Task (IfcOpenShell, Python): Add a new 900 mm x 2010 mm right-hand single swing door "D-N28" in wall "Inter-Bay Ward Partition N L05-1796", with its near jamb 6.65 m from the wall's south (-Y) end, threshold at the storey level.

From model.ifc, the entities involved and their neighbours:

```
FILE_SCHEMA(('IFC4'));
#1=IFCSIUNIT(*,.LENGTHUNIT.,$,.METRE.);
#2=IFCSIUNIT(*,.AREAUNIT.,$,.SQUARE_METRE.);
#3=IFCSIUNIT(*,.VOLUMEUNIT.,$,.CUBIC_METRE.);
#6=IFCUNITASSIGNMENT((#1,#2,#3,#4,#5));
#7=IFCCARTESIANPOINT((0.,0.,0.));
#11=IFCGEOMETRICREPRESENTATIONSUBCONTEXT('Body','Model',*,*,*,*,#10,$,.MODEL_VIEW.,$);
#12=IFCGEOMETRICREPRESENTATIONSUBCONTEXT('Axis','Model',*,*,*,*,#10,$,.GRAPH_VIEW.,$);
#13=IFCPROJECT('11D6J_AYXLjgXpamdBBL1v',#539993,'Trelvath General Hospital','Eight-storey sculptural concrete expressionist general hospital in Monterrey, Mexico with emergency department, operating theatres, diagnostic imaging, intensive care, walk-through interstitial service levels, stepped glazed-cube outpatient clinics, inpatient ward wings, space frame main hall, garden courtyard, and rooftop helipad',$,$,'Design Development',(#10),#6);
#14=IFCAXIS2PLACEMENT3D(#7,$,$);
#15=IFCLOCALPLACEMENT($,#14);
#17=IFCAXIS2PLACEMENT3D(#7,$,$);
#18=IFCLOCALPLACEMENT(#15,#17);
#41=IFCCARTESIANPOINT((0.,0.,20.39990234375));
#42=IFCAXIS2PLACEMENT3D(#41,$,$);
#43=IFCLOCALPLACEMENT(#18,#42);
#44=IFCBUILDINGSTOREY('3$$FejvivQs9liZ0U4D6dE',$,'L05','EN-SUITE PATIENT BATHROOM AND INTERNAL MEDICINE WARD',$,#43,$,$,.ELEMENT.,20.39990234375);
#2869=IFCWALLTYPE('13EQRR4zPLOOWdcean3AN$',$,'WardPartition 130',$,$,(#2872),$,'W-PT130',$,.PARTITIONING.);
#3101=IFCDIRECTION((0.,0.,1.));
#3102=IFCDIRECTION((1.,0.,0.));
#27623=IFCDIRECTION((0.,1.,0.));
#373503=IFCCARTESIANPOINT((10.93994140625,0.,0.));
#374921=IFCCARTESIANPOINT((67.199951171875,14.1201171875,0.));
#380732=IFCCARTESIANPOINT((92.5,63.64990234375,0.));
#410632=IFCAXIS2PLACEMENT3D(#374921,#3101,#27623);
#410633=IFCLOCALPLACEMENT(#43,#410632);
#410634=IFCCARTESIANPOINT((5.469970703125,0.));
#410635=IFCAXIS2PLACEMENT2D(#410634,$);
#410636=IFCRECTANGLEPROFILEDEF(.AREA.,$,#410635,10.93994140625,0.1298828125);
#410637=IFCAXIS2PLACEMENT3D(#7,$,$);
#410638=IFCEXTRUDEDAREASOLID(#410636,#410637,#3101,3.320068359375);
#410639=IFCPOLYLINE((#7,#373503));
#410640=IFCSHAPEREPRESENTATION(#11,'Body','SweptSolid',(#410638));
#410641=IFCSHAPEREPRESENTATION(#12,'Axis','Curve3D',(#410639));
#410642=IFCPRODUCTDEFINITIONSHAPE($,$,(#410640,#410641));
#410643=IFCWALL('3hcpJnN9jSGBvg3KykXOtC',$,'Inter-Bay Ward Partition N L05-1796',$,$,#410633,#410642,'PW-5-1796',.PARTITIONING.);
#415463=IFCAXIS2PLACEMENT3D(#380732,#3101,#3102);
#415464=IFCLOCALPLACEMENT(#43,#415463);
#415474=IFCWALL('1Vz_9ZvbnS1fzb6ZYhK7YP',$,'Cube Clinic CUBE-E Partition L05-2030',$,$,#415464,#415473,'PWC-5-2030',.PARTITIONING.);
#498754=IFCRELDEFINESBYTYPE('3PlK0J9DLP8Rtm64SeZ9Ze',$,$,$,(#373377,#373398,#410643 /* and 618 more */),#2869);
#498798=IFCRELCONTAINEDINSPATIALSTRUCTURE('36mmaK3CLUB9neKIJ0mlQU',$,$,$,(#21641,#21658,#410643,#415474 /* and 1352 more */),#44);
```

```python
import numpy as np
import ifcopenshell
import ifcopenshell.api.feature
import ifcopenshell.api.geometry
import ifcopenshell.api.root
import ifcopenshell.api.spatial
import ifcopenshell.geom
import ifcopenshell.util.element
import ifcopenshell.util.placement
import ifcopenshell.util.representation
import ifcopenshell.util.shape
import ifcopenshell.util.unit

model = ifcopenshell.open("model.ifc")
unit_scale = ifcopenshell.util.unit.calculate_unit_scale(model)
settings = ifcopenshell.geom.settings()


def volume(element):
    """Net volume in cubic metres, openings subtracted."""
    shape = ifcopenshell.geom.create_shape(settings, element)
    return ifcopenshell.util.shape.get_volume(shape.geometry)


wall = model.by_id(410643)
storey = ifcopenshell.util.element.get_container(wall, ifc_class="IfcBuildingStorey")
context = ifcopenshell.util.representation.get_context(model, "Model", "Body", "MODEL_VIEW")
before = volume(wall)

width, height, from_end, sill = 0.9, 2.01, 6.65, 0.0  # metres

# The wall runs along its own X axis, and the end named is its -X end.
wall_shape = ifcopenshell.geom.create_shape(settings, wall)
x, y, z = ifcopenshell.util.shape.get_vertices(wall_shape.geometry).T
start = x.min() + from_end
face, thickness = float(y.min()), float(y.max() - y.min())
wall_matrix = ifcopenshell.util.placement.get_local_placement(wall.ObjectPlacement)
level = ifcopenshell.util.placement.get_local_placement(storey.ObjectPlacement)[2, 3]


def in_wall(x, y):
    """Placement at x, y metres in the wall's axes, at sill height."""
    matrix = wall_matrix.copy()
    matrix[:, 3] = wall_matrix @ np.array([x / unit_scale, y / unit_scale, 0.0, 1.0])
    matrix[2, 3] = level + sill / unit_scale
    return matrix


# Opening: a box that overshoots both wall faces by 50 mm.
opening = ifcopenshell.api.root.create_entity(model, ifc_class="IfcOpeningElement", predefined_type="OPENING")
box = ifcopenshell.api.geometry.add_wall_representation(
    model, context=context, length=width, height=height, thickness=thickness + 0.1
)
ifcopenshell.api.geometry.assign_representation(model, product=opening, representation=box)
ifcopenshell.api.geometry.edit_object_placement(model, product=opening, matrix=in_wall(start, face - 0.05), is_si=False)
ifcopenshell.api.feature.add_feature(model, feature=opening, element=wall)

door = ifcopenshell.api.root.create_entity(model, ifc_class="IfcDoor", name="D-N28", predefined_type="DOOR")
door.OverallWidth, door.OverallHeight = width / unit_scale, height / unit_scale
door.OperationType = "SINGLE_SWING_RIGHT"
body = ifcopenshell.api.geometry.add_door_representation(
    model,
    context=context,
    overall_width=door.OverallWidth,
    overall_height=door.OverallHeight,
    operation_type="SINGLE_SWING_RIGHT",
    lining_properties={"LiningDepth": thickness / unit_scale, "ThresholdDepth": thickness / unit_scale},
)
ifcopenshell.api.geometry.assign_representation(model, product=door, representation=body)
ifcopenshell.api.spatial.assign_container(model, products=[door], relating_structure=storey)
ifcopenshell.api.feature.add_filling(model, opening=opening, element=door)

# The lining spans the wall, so the door starts at the wall face.
ifcopenshell.api.geometry.edit_object_placement(model, product=door, matrix=in_wall(start, face), is_si=False)

after = volume(wall)

print(f"wall volume {before:.3f} -> {after:.3f} m3")

model.write("model_updated.ifc")
```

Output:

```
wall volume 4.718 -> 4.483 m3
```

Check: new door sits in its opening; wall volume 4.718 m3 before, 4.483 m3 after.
